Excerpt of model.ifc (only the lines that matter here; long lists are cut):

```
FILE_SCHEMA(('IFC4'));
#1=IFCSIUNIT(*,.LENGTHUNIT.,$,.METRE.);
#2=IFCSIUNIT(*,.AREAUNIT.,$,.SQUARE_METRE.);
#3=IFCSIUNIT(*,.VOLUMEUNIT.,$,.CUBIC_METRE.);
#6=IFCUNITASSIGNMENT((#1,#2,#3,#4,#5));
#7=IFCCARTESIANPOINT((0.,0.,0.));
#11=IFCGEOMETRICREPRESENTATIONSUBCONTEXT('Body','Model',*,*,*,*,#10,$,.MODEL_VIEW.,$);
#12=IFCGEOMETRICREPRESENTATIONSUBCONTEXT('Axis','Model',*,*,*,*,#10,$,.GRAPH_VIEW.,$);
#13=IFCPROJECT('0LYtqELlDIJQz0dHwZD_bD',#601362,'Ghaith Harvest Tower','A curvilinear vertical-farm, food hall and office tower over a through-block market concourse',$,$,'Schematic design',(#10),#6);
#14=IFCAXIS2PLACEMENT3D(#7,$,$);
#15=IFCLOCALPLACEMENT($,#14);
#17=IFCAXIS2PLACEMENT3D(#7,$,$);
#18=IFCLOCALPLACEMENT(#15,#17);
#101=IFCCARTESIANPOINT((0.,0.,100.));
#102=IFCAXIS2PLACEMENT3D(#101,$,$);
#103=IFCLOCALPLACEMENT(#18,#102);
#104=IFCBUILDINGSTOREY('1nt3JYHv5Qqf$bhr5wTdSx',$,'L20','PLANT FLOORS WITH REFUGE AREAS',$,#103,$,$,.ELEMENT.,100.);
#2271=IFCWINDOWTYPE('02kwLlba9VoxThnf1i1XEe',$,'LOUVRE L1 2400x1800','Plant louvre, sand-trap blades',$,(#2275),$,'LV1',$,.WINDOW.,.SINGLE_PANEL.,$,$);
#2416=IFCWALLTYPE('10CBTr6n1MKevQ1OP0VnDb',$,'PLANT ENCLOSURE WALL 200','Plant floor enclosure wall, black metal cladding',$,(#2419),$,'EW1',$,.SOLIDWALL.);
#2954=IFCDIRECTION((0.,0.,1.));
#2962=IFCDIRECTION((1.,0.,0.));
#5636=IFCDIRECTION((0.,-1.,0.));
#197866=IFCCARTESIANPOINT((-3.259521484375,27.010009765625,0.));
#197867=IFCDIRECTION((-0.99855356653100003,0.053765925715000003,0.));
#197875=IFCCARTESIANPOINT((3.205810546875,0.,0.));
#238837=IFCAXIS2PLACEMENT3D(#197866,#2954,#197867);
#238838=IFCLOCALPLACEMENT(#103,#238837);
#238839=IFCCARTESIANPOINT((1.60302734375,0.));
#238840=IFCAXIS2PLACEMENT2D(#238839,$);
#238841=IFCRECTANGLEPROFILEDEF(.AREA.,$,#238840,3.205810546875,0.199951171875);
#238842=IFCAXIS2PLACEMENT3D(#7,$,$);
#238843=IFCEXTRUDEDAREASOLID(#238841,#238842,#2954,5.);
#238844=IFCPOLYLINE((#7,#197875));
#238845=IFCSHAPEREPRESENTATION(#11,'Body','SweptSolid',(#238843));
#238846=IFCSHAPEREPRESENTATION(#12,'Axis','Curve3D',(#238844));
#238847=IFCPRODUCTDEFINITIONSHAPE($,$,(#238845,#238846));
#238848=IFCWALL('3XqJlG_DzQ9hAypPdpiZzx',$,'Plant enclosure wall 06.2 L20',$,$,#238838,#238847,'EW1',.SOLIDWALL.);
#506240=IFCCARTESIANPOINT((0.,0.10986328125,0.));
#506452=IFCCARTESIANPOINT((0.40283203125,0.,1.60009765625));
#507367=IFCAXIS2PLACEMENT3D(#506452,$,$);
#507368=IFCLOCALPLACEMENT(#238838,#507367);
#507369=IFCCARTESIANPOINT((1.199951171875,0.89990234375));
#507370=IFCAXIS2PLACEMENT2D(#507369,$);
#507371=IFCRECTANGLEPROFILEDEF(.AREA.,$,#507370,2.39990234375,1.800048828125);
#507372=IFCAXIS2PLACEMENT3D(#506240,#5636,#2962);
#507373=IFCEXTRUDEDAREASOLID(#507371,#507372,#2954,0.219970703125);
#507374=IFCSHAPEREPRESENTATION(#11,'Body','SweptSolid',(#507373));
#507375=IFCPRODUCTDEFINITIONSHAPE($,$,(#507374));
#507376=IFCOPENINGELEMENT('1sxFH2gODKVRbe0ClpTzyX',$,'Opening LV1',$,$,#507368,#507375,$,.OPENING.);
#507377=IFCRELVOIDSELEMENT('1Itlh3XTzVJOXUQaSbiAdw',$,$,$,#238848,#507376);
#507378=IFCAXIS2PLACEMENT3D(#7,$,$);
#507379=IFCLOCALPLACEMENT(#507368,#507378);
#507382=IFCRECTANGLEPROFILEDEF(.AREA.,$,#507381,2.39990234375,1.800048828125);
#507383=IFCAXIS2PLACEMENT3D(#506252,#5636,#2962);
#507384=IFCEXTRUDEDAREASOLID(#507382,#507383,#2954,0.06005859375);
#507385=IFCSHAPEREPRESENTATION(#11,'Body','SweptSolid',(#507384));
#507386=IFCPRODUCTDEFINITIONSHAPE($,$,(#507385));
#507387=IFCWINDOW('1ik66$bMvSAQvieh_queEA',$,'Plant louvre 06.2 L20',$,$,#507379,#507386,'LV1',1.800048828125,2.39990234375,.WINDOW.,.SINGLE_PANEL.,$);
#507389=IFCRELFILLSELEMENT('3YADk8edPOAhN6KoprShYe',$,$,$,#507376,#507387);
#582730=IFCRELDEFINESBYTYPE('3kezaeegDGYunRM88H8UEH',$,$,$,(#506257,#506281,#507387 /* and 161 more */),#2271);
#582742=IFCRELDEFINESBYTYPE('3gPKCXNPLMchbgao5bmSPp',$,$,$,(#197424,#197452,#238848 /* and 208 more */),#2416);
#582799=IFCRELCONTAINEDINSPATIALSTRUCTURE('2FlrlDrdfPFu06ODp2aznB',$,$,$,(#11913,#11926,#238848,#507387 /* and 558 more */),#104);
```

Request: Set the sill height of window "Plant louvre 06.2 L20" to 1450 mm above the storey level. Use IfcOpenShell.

```python
import numpy as np
import ifcopenshell
import ifcopenshell.api.geometry
import ifcopenshell.geom
import ifcopenshell.util.element
import ifcopenshell.util.placement
import ifcopenshell.util.shape
import ifcopenshell.util.unit

model = ifcopenshell.open("model.ifc")
unit_scale = ifcopenshell.util.unit.calculate_unit_scale(model)

window = model.by_guid("1ik66$bMvSAQvieh_queEA")
opening = window.FillsVoids[0].RelatingOpeningElement
storey = ifcopenshell.util.element.get_container(window, ifc_class="IfcBuildingStorey")
level = ifcopenshell.util.placement.get_local_placement(storey.ObjectPlacement)[2, 3]

# The opening's origin need not be at the sill, so measure its lowest point.
shape = ifcopenshell.geom.create_shape(ifcopenshell.geom.settings(), opening)
bottom = ifcopenshell.util.shape.get_shape_bottom_elevation(shape, shape.geometry) / unit_scale
dz = level + 1.45 - bottom

shift = np.array([0.0, 0.0, dz])
# The window is placed relative to its opening, so it follows when the opening moves.
matrix = ifcopenshell.util.placement.get_local_placement(opening.ObjectPlacement)
matrix[:3, 3] += shift
ifcopenshell.api.geometry.edit_object_placement(
    model, product=opening, matrix=matrix, is_si=False, should_transform_children=True
)

print(f"moved by {dz * unit_scale:+.3f} m")

model.write("model-out.ifc")
```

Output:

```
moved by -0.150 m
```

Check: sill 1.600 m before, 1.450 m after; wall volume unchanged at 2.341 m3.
